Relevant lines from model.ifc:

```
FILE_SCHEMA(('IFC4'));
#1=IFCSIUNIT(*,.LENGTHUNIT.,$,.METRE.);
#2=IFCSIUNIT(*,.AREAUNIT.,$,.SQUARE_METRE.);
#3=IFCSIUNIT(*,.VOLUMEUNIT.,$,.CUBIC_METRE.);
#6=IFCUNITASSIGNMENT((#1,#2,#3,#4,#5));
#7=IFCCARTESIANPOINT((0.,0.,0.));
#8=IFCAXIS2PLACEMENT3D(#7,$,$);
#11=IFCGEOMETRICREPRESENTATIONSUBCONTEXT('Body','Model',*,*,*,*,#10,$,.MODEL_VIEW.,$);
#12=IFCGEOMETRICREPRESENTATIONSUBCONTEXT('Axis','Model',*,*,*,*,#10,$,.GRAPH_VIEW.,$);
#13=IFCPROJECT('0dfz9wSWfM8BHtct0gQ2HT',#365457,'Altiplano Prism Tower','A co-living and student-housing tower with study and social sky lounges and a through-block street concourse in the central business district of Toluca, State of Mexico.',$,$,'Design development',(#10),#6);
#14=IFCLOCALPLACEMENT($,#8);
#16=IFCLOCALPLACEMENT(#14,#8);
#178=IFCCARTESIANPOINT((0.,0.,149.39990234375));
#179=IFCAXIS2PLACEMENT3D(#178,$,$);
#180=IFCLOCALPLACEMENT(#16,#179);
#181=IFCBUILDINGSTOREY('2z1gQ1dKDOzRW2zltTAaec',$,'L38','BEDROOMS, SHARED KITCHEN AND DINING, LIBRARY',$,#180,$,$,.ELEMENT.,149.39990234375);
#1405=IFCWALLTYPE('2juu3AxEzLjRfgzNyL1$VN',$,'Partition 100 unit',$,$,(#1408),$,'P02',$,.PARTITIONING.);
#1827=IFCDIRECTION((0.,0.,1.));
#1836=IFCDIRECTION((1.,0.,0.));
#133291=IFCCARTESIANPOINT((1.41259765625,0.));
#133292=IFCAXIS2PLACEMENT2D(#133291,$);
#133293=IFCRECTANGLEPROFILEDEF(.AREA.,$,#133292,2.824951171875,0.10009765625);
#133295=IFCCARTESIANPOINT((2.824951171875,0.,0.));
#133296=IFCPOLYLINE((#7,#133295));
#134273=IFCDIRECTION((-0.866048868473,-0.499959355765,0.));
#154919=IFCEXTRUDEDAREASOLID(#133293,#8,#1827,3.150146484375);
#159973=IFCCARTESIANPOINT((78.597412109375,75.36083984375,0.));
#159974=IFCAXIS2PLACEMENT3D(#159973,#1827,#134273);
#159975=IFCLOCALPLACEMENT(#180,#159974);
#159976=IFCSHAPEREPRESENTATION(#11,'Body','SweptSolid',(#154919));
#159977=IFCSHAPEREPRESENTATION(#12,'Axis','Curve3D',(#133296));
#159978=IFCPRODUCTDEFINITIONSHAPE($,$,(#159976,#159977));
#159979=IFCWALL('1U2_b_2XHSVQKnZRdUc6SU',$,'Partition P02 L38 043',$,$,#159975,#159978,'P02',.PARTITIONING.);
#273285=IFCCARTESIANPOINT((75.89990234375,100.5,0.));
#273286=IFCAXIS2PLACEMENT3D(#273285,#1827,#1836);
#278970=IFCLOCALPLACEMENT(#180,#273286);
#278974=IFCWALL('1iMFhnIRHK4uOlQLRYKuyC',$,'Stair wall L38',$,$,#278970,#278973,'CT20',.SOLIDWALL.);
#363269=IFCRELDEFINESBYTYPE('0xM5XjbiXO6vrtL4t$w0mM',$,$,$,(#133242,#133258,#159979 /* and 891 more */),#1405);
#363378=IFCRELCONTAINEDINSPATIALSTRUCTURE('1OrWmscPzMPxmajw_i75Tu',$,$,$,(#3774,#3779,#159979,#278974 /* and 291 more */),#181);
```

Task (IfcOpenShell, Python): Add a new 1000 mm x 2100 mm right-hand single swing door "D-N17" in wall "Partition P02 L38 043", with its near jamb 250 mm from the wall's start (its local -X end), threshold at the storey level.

```python
import numpy as np
import ifcopenshell
import ifcopenshell.api.feature
import ifcopenshell.api.geometry
import ifcopenshell.api.root
import ifcopenshell.api.spatial
import ifcopenshell.geom
import ifcopenshell.util.element
import ifcopenshell.util.placement
import ifcopenshell.util.representation
import ifcopenshell.util.shape
import ifcopenshell.util.unit

model = ifcopenshell.open("model.ifc")
unit_scale = ifcopenshell.util.unit.calculate_unit_scale(model)
settings = ifcopenshell.geom.settings()


def volume(element):
    """Net volume in cubic metres, openings subtracted."""
    shape = ifcopenshell.geom.create_shape(settings, element)
    return ifcopenshell.util.shape.get_volume(shape.geometry)


wall = model.by_guid("1U2_b_2XHSVQKnZRdUc6SU")
storey = ifcopenshell.util.element.get_container(wall, ifc_class="IfcBuildingStorey")
context = ifcopenshell.util.representation.get_context(model, "Model", "Body", "MODEL_VIEW")
before = volume(wall)

width, height, from_end, sill = 1, 2.1, 0.25, 0.0  # metres

# The wall runs along its own X axis, and the end named is its -X end.
wall_shape = ifcopenshell.geom.create_shape(settings, wall)
x, y, z = ifcopenshell.util.shape.get_vertices(wall_shape.geometry).T
start = x.min() + from_end
face, thickness = float(y.min()), float(y.max() - y.min())
wall_matrix = ifcopenshell.util.placement.get_local_placement(wall.ObjectPlacement)
level = ifcopenshell.util.placement.get_local_placement(storey.ObjectPlacement)[2, 3]


def in_wall(x, y):
    """Placement at x, y metres in the wall's axes, at sill height."""
    matrix = wall_matrix.copy()
    matrix[:, 3] = wall_matrix @ np.array([x / unit_scale, y / unit_scale, 0.0, 1.0])
    matrix[2, 3] = level + sill / unit_scale
    return matrix


# Opening: a box that overshoots both wall faces by 50 mm.
opening = ifcopenshell.api.root.create_entity(model, ifc_class="IfcOpeningElement", predefined_type="OPENING")
box = ifcopenshell.api.geometry.add_wall_representation(
    model, context=context, length=width, height=height, thickness=thickness + 0.1
)
ifcopenshell.api.geometry.assign_representation(model, product=opening, representation=box)
ifcopenshell.api.geometry.edit_object_placement(model, product=opening, matrix=in_wall(start, face - 0.05), is_si=False)
ifcopenshell.api.feature.add_feature(model, feature=opening, element=wall)

door = ifcopenshell.api.root.create_entity(model, ifc_class="IfcDoor", name="D-N17", predefined_type="DOOR")
door.OverallWidth, door.OverallHeight = width / unit_scale, height / unit_scale
door.OperationType = "SINGLE_SWING_RIGHT"
body = ifcopenshell.api.geometry.add_door_representation(
    model,
    context=context,
    overall_width=door.OverallWidth,
    overall_height=door.OverallHeight,
    operation_type="SINGLE_SWING_RIGHT",
    lining_properties={"LiningDepth": thickness / unit_scale, "ThresholdDepth": thickness / unit_scale},
)
ifcopenshell.api.geometry.assign_representation(model, product=door, representation=body)
ifcopenshell.api.spatial.assign_container(model, products=[door], relating_structure=storey)
ifcopenshell.api.feature.add_filling(model, opening=opening, element=door)

# The lining spans the wall, so the door starts at the wall face.
ifcopenshell.api.geometry.edit_object_placement(model, product=door, matrix=in_wall(start, face), is_si=False)

after = volume(wall)

print(f"wall volume {before:.3f} -> {after:.3f} m3")

model.write("model_edited.ifc")
```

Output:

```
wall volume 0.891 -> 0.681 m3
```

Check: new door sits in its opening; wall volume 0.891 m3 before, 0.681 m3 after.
